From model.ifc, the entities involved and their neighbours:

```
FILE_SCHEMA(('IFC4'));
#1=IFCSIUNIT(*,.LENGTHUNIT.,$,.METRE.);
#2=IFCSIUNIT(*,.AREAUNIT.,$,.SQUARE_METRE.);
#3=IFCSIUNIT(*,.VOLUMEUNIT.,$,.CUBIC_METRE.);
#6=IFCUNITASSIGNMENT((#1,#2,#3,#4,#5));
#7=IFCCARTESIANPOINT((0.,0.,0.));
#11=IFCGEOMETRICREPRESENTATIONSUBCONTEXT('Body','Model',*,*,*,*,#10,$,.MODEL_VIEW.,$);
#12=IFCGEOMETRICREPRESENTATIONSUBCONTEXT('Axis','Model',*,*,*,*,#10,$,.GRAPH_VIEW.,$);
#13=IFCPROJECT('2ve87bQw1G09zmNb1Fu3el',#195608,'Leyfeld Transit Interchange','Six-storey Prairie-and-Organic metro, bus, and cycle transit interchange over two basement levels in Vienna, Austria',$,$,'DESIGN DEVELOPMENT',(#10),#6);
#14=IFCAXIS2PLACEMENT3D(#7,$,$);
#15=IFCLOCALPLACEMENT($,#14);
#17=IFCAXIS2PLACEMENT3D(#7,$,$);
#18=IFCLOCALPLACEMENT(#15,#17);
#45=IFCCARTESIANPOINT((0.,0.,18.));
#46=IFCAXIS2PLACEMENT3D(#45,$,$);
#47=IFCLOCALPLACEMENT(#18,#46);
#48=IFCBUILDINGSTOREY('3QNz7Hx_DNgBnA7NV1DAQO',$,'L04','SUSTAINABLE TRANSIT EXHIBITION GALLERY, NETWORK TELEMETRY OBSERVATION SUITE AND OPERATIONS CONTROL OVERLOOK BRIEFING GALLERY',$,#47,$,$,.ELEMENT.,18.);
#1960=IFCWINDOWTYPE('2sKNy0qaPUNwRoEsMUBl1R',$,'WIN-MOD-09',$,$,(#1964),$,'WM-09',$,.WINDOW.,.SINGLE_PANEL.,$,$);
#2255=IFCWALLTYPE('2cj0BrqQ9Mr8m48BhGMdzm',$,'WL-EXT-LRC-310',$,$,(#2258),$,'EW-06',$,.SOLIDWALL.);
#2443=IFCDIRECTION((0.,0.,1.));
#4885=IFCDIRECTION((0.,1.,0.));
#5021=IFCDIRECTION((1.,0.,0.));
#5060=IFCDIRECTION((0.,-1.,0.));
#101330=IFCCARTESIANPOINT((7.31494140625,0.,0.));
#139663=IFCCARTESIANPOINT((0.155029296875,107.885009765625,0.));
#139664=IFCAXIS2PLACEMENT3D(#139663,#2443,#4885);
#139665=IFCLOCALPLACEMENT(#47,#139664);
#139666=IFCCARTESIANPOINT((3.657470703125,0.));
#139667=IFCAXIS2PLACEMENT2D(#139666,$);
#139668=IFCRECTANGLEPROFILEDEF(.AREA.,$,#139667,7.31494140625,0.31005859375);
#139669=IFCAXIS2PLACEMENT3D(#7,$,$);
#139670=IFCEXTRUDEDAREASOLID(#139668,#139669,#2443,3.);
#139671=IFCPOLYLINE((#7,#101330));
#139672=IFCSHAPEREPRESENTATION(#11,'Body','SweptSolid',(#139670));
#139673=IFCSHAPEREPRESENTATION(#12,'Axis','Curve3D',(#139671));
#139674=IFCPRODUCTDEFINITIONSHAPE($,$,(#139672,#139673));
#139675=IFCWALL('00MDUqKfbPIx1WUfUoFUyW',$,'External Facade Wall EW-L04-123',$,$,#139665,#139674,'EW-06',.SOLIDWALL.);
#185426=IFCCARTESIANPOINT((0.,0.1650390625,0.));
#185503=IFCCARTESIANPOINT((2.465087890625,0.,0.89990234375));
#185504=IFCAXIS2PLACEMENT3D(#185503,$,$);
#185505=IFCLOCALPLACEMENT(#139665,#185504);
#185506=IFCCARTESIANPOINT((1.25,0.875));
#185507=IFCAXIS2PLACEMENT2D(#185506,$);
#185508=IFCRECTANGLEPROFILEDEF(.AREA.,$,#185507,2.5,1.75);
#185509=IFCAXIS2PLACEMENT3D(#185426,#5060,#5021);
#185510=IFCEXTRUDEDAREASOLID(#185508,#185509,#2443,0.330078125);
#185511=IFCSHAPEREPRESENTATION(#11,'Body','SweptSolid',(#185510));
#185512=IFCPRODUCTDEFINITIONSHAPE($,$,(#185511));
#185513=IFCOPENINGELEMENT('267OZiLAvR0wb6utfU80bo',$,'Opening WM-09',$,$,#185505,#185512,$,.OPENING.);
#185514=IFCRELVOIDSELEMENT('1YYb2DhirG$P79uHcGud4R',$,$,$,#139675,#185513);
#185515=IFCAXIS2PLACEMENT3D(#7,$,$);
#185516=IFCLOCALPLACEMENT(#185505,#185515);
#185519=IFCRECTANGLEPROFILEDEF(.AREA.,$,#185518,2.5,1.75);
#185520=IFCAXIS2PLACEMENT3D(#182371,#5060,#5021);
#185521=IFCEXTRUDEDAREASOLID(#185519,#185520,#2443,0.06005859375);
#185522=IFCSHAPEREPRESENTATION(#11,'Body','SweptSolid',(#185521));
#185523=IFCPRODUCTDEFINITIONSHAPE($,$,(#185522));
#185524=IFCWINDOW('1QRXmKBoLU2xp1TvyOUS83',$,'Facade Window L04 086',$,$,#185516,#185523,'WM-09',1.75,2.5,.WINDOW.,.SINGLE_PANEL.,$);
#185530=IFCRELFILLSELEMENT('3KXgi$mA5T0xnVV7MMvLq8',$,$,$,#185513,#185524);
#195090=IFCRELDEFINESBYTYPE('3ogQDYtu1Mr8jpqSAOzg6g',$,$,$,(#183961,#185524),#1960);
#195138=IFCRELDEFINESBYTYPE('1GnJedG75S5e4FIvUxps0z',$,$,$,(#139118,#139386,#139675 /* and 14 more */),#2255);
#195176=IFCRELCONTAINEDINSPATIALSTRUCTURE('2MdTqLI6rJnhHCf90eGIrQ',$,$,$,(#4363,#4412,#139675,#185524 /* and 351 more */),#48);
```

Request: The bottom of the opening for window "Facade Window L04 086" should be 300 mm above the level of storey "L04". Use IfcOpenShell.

```python
import numpy as np
import ifcopenshell
import ifcopenshell.api.geometry
import ifcopenshell.geom
import ifcopenshell.util.element
import ifcopenshell.util.placement
import ifcopenshell.util.shape
import ifcopenshell.util.unit

model = ifcopenshell.open("model.ifc")
unit_scale = ifcopenshell.util.unit.calculate_unit_scale(model)

window = model.by_id(185524)
opening = window.FillsVoids[0].RelatingOpeningElement
storey = ifcopenshell.util.element.get_container(window, ifc_class="IfcBuildingStorey")
level = ifcopenshell.util.placement.get_local_placement(storey.ObjectPlacement)[2, 3]

# The opening's origin need not be at the sill, so measure its lowest point.
shape = ifcopenshell.geom.create_shape(ifcopenshell.geom.settings(), opening)
bottom = ifcopenshell.util.shape.get_shape_bottom_elevation(shape, shape.geometry) / unit_scale
dz = level + 0.3 / unit_scale - bottom

shift = np.array([0.0, 0.0, dz])
# The window is placed relative to its opening, so it follows when the opening moves.
matrix = ifcopenshell.util.placement.get_local_placement(opening.ObjectPlacement)
matrix[:3, 3] += shift
ifcopenshell.api.geometry.edit_object_placement(
    model, product=opening, matrix=matrix, is_si=False, should_transform_children=True
)

print(f"moved by {dz * unit_scale:+.3f} m")

model.write("model_v2.ifc")
```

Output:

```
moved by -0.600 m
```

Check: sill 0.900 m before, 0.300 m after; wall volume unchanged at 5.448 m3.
